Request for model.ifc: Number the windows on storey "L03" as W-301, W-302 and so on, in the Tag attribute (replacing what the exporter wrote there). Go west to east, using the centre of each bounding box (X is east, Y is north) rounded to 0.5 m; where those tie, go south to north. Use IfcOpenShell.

First a look at what the model holds.

```python
import ifcopenshell
import ifcopenshell.util.element
import ifcopenshell.util.placement

model = ifcopenshell.open("model.ifc")
print(model.schema)
storey = next(s for s in model.by_type("IfcBuildingStorey") if s.Name == "L03")
windows = [e for e in ifcopenshell.util.element.get_decomposition(storey) if e.is_a("IfcWindow")]
for e in sorted(windows, key=lambda e: e.id()):
    origin = ifcopenshell.util.placement.get_local_placement(e.ObjectPlacement)[:3, 3]
    print(e.id(), e.Tag, e.Name, origin.round(2) + 0.0, sep=" | ")
```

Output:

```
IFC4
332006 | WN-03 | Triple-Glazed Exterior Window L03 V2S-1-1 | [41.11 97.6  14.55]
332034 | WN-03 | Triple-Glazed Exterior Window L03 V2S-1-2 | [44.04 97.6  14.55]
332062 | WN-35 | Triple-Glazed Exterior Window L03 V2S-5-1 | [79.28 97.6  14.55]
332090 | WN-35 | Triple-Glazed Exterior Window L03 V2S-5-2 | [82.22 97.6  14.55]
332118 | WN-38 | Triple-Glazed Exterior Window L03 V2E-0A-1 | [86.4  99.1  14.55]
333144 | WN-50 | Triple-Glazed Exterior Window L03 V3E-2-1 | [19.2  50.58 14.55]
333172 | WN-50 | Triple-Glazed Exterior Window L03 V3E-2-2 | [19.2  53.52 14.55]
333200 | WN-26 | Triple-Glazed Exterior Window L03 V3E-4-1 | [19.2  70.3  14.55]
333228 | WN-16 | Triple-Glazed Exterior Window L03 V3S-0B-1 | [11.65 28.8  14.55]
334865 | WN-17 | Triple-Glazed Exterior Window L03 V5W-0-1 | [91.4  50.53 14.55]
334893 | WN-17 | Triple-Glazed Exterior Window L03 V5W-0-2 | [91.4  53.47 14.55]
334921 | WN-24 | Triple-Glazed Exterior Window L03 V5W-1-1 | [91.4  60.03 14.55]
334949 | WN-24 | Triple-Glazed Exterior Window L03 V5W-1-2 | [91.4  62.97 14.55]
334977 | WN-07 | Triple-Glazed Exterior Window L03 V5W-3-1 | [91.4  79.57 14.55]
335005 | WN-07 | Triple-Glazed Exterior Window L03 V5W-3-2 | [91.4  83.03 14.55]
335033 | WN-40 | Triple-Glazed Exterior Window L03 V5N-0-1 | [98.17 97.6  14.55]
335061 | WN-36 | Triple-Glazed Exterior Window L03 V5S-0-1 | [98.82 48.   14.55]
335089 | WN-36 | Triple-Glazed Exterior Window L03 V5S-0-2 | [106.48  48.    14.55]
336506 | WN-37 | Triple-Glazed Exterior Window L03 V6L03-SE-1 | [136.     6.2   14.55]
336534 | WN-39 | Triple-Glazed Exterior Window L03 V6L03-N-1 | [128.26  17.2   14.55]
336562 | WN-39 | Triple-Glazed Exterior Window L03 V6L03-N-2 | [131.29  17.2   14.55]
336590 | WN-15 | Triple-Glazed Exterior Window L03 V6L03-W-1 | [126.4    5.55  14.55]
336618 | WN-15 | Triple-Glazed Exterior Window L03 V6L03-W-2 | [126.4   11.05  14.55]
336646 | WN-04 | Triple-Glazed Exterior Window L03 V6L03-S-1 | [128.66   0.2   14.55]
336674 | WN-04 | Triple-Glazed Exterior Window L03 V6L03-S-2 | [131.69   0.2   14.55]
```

```python
import ifcopenshell
import ifcopenshell.geom
import ifcopenshell.util.element
import ifcopenshell.util.shape

model = ifcopenshell.open("model.ifc")
settings = ifcopenshell.geom.settings()
settings.set("use-world-coords", True)


def centre(element):
    shape = ifcopenshell.geom.create_shape(settings, element)
    return ifcopenshell.util.shape.get_bbox_centroid(shape.geometry)


storey = next(s for s in model.by_type("IfcBuildingStorey") if s.Name == "L03")
windows = [e for e in ifcopenshell.util.element.get_decomposition(storey) if e.is_a("IfcWindow")]

# Insertion points can sit at a corner or the storey origin, so sort by the geometry (in metres).
centres = {e: centre(e) for e in windows}
windows.sort(key=lambda e: (round(centres[e][0] / 0.5), centres[e][1]))

for i, e in enumerate(windows, start=1):
    number = f"W-3{i:02d}"
    e.Tag = number
    print(e.id(), number)

model.write("model_v2.ifc")
```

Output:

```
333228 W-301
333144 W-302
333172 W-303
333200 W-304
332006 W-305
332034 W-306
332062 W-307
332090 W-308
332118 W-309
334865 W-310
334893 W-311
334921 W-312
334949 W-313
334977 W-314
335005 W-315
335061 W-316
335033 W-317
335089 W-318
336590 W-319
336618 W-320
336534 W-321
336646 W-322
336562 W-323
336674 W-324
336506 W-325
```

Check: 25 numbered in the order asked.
